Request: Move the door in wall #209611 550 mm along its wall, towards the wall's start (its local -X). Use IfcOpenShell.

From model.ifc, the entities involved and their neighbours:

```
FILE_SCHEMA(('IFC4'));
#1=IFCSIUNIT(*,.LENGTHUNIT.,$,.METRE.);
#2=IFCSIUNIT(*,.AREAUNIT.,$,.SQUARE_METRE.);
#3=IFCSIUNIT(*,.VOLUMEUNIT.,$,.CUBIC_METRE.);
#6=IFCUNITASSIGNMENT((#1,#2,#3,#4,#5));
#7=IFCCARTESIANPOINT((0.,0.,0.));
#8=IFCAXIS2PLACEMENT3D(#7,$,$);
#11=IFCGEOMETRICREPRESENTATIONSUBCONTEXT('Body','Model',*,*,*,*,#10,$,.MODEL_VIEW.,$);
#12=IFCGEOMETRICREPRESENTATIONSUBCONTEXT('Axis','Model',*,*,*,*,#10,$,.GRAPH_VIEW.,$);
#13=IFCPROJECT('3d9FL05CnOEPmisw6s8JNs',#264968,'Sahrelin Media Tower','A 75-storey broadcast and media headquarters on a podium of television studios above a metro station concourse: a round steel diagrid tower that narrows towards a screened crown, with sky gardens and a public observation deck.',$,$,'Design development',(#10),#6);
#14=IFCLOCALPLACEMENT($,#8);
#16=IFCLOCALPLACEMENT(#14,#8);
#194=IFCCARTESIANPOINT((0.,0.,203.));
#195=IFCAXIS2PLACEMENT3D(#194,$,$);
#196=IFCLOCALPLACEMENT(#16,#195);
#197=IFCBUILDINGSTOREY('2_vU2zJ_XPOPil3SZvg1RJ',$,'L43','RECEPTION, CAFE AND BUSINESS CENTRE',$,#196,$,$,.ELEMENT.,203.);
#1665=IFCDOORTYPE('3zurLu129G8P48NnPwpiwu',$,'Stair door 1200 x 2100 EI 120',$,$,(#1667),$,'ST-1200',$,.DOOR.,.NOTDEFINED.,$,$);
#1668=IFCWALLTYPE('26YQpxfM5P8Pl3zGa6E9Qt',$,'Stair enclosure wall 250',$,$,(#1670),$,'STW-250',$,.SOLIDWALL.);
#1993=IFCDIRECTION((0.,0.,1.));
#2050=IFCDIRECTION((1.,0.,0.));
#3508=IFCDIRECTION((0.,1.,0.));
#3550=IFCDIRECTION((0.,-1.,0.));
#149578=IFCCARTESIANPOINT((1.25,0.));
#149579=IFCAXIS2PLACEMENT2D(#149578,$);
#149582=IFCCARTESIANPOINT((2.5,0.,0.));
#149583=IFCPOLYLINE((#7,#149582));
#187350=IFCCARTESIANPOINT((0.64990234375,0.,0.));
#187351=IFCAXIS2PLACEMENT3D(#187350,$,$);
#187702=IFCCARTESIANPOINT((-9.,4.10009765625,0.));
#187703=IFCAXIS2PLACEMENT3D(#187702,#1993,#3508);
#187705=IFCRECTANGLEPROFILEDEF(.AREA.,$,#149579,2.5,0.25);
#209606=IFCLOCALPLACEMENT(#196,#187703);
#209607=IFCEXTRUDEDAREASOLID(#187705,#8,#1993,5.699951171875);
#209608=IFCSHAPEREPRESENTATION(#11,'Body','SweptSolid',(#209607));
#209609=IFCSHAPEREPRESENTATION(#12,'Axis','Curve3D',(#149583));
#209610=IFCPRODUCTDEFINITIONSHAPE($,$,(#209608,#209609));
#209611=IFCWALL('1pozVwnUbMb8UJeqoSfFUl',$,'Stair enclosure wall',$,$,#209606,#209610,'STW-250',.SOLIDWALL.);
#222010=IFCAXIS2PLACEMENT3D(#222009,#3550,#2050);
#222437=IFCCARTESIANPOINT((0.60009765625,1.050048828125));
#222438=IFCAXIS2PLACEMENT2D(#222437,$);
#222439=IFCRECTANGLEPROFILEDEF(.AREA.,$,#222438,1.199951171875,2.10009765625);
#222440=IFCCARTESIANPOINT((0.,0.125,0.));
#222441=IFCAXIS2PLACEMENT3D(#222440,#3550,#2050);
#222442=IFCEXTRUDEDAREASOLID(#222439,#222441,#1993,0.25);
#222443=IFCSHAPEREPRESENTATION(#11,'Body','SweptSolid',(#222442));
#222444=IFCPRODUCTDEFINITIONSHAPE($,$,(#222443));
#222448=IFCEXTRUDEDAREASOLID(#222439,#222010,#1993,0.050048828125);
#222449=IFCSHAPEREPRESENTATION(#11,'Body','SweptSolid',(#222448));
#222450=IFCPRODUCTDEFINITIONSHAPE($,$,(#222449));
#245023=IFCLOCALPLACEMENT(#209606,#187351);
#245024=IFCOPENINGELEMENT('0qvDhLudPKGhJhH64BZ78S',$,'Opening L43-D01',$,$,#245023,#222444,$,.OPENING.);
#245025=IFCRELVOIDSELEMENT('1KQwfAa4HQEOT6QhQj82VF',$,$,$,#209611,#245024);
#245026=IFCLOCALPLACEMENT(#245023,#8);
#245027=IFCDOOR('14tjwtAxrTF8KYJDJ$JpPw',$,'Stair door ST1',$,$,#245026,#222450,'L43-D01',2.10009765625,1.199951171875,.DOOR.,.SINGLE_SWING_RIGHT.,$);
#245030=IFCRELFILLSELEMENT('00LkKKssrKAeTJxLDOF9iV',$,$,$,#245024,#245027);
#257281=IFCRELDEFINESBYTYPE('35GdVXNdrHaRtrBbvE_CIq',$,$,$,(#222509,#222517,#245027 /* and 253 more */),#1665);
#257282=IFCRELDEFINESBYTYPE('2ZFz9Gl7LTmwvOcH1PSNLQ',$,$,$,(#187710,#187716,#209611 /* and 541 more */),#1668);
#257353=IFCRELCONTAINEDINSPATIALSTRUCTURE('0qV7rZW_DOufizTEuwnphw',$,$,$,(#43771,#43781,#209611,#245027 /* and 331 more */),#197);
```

```python
import ifcopenshell
import ifcopenshell.api.geometry
import ifcopenshell.util.placement
import ifcopenshell.util.unit

model = ifcopenshell.open("model.ifc")
unit_scale = ifcopenshell.util.unit.calculate_unit_scale(model)

door = model.by_guid("14tjwtAxrTF8KYJDJ$JpPw")
opening = door.FillsVoids[0].RelatingOpeningElement
wall = opening.VoidsElements[0].RelatingBuildingElement

wall_matrix = ifcopenshell.util.placement.get_local_placement(wall.ObjectPlacement)
shift = wall_matrix[:3, 0] * -0.55 / unit_scale
before = ifcopenshell.util.placement.get_local_placement(door.ObjectPlacement)[:3, 3].copy()

# The door is placed relative to its opening, so it follows when the opening moves.
matrix = ifcopenshell.util.placement.get_local_placement(opening.ObjectPlacement)
matrix[:3, 3] += shift
ifcopenshell.api.geometry.edit_object_placement(
    model, product=opening, matrix=matrix, is_si=False, should_transform_children=True
)

after = ifcopenshell.util.placement.get_local_placement(door.ObjectPlacement)[:3, 3]
print("door moved by", (after - before).round(3) + 0.0)

model.write("model-out.ifc")
```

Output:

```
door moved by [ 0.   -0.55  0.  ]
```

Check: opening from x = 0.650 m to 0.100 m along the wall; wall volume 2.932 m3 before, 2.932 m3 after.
